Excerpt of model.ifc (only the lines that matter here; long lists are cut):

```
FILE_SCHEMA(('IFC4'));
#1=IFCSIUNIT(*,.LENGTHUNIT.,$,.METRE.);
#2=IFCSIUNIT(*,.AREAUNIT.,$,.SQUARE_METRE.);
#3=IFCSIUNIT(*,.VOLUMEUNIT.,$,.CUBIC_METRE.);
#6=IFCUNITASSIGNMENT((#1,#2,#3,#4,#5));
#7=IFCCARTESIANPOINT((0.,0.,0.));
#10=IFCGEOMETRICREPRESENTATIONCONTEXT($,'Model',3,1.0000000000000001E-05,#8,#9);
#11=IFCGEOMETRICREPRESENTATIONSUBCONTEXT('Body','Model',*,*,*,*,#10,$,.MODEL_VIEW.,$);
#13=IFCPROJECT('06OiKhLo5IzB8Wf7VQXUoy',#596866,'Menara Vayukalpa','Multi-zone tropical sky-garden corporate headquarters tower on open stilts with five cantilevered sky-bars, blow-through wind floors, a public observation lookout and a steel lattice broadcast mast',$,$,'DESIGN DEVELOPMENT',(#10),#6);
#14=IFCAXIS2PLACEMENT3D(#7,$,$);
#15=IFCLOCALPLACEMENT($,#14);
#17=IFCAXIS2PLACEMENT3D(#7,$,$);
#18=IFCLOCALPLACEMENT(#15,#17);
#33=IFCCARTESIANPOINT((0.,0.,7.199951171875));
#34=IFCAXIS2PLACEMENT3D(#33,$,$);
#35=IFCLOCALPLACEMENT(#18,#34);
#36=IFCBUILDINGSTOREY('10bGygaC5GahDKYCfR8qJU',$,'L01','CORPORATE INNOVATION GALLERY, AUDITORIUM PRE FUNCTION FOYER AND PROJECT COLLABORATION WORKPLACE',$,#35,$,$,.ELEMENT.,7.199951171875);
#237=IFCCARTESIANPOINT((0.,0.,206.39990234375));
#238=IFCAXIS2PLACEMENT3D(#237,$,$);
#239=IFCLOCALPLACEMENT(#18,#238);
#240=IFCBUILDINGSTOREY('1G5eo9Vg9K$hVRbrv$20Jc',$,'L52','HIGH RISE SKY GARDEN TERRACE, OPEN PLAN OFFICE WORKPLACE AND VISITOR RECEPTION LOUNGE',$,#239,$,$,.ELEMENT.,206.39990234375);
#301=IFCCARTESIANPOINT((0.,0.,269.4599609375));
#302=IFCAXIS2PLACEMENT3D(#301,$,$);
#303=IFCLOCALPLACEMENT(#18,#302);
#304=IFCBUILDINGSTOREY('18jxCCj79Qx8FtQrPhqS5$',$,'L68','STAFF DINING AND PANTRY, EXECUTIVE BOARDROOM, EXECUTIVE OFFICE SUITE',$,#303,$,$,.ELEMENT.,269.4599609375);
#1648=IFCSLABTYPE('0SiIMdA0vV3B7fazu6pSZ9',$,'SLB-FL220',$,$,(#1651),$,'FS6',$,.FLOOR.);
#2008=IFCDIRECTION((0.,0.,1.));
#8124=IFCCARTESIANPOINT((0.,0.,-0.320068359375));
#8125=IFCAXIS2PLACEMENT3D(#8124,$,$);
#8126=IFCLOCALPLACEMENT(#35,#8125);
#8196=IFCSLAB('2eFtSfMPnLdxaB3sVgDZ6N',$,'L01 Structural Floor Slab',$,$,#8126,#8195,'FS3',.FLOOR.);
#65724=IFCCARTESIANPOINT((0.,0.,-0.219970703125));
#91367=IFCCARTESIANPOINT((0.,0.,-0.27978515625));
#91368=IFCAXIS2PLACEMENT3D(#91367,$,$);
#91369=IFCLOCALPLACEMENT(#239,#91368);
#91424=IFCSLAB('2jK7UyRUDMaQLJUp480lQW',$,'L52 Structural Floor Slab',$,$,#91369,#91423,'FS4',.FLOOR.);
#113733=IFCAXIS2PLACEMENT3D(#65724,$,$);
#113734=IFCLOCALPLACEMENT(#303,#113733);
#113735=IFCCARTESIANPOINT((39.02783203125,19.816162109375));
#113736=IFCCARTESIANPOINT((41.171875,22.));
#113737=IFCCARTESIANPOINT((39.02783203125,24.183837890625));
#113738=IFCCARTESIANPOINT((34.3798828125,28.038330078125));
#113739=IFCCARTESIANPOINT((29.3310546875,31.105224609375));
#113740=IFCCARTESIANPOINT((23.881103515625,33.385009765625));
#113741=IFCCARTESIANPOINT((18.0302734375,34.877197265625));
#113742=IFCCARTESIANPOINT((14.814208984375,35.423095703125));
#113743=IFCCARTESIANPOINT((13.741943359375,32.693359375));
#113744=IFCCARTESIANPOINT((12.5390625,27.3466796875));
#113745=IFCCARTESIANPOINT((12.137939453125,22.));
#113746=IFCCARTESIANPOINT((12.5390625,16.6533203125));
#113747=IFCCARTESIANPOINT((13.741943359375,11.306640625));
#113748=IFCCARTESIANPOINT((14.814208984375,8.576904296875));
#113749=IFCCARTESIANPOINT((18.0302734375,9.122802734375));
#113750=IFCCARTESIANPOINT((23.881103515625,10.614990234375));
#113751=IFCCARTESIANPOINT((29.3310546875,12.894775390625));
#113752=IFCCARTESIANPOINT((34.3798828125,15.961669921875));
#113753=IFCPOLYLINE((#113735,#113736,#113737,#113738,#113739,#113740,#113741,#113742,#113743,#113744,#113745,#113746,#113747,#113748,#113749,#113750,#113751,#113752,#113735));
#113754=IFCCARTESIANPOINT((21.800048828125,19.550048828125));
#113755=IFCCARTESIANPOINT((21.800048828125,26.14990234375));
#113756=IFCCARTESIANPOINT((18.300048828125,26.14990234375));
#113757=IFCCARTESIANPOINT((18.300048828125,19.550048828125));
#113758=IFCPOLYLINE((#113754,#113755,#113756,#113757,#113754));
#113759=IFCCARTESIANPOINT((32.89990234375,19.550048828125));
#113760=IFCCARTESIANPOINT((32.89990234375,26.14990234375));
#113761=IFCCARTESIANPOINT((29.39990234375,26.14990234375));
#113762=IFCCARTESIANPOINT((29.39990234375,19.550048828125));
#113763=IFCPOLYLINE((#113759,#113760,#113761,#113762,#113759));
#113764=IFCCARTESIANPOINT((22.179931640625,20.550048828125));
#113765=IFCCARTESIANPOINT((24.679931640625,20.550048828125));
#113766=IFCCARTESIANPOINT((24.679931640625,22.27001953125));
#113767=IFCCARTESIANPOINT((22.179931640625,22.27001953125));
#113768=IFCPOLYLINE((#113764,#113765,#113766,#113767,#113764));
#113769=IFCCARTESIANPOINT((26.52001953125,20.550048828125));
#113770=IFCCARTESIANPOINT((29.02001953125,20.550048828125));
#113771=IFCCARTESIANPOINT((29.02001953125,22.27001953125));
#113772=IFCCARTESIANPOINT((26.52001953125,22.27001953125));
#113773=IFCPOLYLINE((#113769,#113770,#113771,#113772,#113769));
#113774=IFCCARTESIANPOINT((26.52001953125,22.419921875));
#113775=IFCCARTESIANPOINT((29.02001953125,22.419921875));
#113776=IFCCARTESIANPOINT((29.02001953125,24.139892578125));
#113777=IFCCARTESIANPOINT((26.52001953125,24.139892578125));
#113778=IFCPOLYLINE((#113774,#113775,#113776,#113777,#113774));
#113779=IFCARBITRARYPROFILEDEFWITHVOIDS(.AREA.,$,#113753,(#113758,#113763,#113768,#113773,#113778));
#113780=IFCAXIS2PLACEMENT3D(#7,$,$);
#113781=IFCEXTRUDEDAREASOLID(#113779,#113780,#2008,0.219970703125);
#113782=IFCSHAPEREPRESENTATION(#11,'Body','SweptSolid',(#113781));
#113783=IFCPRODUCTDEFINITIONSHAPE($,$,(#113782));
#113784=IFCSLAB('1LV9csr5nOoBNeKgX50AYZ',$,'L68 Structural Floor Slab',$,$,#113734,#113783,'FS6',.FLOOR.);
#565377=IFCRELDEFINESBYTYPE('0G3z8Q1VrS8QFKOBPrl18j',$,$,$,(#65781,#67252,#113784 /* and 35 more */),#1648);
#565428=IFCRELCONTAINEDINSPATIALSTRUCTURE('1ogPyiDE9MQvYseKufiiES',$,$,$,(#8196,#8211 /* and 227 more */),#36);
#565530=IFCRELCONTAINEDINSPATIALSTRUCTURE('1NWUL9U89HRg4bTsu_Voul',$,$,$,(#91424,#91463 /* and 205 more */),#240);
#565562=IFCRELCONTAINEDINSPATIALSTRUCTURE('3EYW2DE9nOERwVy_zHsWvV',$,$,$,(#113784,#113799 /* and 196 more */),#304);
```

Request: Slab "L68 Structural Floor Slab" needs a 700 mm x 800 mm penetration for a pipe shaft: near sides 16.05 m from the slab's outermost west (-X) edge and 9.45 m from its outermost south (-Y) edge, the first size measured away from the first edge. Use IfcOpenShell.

```python
import numpy as np
import ifcopenshell
import ifcopenshell.api.feature
import ifcopenshell.api.geometry
import ifcopenshell.api.root
import ifcopenshell.geom
import ifcopenshell.util.placement
import ifcopenshell.util.representation
import ifcopenshell.util.shape
import ifcopenshell.util.unit

model = ifcopenshell.open("model.ifc")
unit_scale = ifcopenshell.util.unit.calculate_unit_scale(model)
settings = ifcopenshell.geom.settings()


def volume(element):
    """Net volume in cubic metres, openings subtracted."""
    shape = ifcopenshell.geom.create_shape(settings, element)
    return ifcopenshell.util.shape.get_volume(shape.geometry)


slab = model.by_guid("1LV9csr5nOoBNeKgX50AYZ")
before = volume(slab)

# Extent in the slab's own axes, in metres. The edges named are its -X and -Y sides.
slab_shape = ifcopenshell.geom.create_shape(settings, slab)
vertices = ifcopenshell.util.shape.get_vertices(slab_shape.geometry)
x_min, y_min, bottom = vertices.min(axis=0)
top = vertices[:, 2].max()

opening = ifcopenshell.api.root.create_entity(model, ifc_class="IfcOpeningElement", name="Pipe shaft opening", predefined_type="OPENING")
context = ifcopenshell.util.representation.get_context(model, "Model", "Body", "MODEL_VIEW")
width, depth = 0.7, 0.8
outline = [(0.0, 0.0), (width, 0.0), (width, depth), (0.0, depth), (0.0, 0.0)]
# Overshoot both faces by 50 mm so the cut is clean.
shape = ifcopenshell.api.geometry.add_slab_representation(
    model, context=context, depth=top - bottom + 0.1, polyline=outline
)
ifcopenshell.api.geometry.assign_representation(model, product=opening, representation=shape)

matrix = ifcopenshell.util.placement.get_local_placement(slab.ObjectPlacement)
matrix[:, 3] = matrix @ np.append(np.array([x_min + 16.05, y_min + 9.45, bottom - 0.05]) / unit_scale, 1.0)
ifcopenshell.api.geometry.edit_object_placement(model, product=opening, matrix=matrix, is_si=False)
ifcopenshell.api.feature.add_feature(model, feature=opening, element=slab)

after = volume(slab)

print(f"slab volume {before:.3f} -> {after:.3f} m3")

model.write("model_updated.ifc")
```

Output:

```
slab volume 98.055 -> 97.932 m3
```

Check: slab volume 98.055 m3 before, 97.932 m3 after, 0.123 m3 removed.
